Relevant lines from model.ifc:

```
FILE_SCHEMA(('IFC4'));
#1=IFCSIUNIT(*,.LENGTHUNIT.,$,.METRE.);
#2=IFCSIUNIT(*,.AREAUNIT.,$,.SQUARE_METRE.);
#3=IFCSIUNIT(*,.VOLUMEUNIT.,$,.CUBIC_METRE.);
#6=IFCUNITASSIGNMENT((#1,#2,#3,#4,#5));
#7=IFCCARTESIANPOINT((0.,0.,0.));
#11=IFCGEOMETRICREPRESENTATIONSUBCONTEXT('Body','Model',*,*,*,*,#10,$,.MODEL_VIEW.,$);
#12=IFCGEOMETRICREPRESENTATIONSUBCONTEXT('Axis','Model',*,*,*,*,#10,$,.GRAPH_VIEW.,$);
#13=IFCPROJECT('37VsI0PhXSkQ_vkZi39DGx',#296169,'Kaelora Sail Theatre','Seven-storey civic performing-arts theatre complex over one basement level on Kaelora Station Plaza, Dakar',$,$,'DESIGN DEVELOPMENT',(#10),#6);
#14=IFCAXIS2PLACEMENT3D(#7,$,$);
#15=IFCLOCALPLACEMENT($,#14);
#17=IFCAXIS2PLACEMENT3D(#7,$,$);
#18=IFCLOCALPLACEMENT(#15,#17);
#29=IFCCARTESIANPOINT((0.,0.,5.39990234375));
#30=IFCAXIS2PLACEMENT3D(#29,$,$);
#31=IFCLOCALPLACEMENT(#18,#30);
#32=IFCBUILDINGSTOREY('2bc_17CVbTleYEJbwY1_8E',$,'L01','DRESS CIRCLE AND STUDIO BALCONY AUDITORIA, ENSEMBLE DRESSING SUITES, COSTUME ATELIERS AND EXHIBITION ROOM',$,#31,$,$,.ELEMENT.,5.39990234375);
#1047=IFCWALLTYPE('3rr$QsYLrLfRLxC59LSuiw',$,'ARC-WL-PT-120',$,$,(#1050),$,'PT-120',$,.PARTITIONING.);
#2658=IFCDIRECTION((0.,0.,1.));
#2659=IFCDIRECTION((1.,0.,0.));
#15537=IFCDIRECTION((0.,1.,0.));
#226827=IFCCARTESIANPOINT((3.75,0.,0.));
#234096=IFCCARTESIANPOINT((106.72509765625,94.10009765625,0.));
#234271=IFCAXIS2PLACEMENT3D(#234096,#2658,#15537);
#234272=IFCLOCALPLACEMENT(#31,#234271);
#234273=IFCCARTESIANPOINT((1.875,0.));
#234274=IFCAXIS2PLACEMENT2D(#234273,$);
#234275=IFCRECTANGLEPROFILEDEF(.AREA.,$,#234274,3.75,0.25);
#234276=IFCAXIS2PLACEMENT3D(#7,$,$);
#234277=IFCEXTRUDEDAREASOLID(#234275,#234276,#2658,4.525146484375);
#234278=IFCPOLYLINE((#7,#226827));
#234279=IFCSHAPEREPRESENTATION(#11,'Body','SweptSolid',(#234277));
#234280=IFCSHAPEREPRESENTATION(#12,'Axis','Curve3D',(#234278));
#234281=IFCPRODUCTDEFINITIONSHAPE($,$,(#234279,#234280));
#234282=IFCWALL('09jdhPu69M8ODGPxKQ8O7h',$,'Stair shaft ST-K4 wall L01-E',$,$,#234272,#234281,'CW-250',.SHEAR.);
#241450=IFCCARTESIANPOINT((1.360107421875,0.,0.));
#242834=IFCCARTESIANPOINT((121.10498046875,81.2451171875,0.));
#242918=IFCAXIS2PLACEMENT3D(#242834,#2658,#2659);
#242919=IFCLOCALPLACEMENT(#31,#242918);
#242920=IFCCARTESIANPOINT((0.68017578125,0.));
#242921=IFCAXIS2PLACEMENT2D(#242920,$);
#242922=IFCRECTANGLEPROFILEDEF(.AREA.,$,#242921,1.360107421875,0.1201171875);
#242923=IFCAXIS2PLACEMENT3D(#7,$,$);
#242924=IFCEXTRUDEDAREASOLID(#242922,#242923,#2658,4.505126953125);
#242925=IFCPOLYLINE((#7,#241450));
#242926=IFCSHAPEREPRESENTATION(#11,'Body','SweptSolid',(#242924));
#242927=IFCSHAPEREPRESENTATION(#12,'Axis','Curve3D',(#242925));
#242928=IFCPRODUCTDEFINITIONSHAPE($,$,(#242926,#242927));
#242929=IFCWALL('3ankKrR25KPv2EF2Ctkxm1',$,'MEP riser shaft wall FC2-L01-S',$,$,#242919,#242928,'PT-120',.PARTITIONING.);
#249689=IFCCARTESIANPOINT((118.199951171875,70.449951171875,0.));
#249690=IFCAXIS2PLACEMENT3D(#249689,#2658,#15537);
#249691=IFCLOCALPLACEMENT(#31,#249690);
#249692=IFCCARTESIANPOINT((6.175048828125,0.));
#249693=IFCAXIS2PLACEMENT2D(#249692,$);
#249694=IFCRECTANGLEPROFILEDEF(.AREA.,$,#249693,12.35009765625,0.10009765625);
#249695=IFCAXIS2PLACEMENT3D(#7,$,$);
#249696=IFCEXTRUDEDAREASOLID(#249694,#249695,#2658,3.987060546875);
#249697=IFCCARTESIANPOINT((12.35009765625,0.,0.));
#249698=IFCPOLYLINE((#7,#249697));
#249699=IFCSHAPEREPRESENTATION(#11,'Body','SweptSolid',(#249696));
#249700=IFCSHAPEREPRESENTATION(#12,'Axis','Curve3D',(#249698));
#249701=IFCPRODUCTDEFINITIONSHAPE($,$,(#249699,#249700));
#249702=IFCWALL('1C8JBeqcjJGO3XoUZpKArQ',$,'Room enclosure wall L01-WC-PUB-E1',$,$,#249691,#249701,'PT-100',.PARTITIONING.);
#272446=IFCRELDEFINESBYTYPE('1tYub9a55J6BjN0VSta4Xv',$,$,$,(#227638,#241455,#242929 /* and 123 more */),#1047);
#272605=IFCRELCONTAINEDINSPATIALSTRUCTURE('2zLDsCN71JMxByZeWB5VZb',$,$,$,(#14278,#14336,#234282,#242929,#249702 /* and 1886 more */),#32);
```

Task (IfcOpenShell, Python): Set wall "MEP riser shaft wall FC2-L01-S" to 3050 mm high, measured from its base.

```python
import ifcopenshell
import ifcopenshell.geom
import ifcopenshell.util.representation
import ifcopenshell.util.shape

model = ifcopenshell.open("model.ifc")
settings = ifcopenshell.geom.settings()


def volume(element):
    """Net volume in cubic metres, openings subtracted."""
    shape = ifcopenshell.geom.create_shape(settings, element)
    return ifcopenshell.util.shape.get_volume(shape.geometry)


wall = model.by_guid("3ankKrR25KPv2EF2Ctkxm1")
before = volume(wall)

body = ifcopenshell.util.representation.get_representation(wall, "Model", "Body")
solid = body.Items[0]
old_height = solid.Depth
solid.Depth = 3.05
after = volume(wall)

print(f"height {old_height:g} -> {solid.Depth:g}, volume {before:.3f} -> {after:.3f} m3")

model.write("model-out.ifc")
```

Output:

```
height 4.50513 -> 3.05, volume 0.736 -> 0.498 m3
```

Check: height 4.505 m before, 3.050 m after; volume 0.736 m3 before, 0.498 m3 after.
